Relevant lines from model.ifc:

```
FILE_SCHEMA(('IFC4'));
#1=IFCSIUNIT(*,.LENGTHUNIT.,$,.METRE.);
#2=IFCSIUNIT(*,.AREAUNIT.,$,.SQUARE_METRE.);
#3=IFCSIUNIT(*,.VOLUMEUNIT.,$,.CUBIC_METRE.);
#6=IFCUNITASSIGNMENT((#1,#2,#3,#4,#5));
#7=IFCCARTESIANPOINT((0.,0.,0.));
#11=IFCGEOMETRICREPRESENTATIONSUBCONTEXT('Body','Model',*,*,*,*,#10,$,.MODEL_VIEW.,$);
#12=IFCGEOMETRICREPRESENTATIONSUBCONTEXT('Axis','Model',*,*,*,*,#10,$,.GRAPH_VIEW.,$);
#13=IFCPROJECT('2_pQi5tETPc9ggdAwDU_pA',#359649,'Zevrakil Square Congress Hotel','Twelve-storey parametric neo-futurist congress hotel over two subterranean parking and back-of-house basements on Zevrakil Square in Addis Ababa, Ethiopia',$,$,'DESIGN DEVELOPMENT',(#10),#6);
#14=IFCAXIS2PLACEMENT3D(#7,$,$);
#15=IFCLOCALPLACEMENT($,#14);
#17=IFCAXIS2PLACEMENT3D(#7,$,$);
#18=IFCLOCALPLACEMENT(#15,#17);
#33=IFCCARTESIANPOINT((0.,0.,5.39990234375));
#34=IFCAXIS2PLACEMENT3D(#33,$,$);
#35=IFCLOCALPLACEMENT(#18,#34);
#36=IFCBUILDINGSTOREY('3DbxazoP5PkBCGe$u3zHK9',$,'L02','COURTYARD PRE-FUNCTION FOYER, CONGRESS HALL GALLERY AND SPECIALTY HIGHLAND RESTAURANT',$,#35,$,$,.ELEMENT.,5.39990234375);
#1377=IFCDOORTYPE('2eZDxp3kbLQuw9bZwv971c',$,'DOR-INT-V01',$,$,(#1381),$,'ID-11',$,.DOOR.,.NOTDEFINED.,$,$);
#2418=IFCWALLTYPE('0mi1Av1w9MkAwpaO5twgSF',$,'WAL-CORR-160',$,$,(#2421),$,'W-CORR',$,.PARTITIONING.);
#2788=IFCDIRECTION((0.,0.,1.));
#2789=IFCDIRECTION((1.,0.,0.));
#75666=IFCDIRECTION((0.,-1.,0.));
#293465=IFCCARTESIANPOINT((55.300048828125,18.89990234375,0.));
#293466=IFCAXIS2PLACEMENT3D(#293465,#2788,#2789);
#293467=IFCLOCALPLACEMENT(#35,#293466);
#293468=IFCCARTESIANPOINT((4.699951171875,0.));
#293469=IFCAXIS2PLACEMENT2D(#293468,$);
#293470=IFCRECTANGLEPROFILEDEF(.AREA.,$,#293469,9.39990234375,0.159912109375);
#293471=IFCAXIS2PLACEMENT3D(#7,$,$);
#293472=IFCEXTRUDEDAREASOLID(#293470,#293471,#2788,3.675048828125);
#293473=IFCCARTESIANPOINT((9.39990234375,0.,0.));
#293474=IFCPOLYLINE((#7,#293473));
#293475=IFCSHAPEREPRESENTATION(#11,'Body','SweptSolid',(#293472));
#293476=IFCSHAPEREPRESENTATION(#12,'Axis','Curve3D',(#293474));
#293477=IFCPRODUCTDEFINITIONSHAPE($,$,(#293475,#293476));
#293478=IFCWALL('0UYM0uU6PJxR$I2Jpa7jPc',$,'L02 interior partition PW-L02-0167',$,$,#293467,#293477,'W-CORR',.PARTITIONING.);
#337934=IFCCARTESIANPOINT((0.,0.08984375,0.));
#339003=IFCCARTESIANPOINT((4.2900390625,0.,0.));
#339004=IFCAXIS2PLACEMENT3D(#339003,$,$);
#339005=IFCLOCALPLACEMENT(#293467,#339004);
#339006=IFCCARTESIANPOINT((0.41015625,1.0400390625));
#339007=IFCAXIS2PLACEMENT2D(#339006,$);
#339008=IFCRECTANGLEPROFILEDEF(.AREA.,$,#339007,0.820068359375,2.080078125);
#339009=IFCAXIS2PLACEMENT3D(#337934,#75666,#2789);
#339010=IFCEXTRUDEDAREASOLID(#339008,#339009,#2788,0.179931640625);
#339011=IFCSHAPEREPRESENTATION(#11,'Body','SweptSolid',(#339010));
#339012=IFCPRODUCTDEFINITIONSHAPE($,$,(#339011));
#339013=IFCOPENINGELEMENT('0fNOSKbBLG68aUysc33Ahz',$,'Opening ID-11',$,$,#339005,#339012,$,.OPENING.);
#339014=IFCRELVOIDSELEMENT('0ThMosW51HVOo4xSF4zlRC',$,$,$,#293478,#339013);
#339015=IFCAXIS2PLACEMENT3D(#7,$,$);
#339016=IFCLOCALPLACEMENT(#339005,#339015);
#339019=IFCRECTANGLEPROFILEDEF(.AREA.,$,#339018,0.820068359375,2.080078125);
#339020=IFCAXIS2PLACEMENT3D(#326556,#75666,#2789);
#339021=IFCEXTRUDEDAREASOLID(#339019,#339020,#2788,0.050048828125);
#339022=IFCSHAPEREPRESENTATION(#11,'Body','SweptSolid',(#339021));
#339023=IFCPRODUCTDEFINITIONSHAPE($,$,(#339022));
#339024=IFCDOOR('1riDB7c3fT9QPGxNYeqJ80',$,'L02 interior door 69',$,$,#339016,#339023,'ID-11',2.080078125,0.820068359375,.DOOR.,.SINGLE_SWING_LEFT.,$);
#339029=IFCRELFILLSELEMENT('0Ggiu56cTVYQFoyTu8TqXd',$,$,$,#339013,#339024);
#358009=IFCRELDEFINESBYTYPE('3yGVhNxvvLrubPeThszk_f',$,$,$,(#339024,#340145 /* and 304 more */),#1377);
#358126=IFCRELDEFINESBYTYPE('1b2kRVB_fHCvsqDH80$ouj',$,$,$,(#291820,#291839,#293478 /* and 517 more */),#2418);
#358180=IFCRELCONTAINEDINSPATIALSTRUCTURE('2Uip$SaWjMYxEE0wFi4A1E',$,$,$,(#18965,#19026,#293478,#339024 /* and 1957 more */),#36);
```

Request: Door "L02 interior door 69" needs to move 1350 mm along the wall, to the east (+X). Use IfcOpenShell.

```python
import ifcopenshell
import ifcopenshell.api.geometry
import ifcopenshell.util.placement

model = ifcopenshell.open("model.ifc")

door = model.by_id(339024)
opening = door.FillsVoids[0].RelatingOpeningElement
wall = opening.VoidsElements[0].RelatingBuildingElement

wall_matrix = ifcopenshell.util.placement.get_local_placement(wall.ObjectPlacement)
shift = wall_matrix[:3, 0] * 1.35
before = ifcopenshell.util.placement.get_local_placement(door.ObjectPlacement)[:3, 3].copy()

# The door is placed relative to its opening, so it follows when the opening moves.
matrix = ifcopenshell.util.placement.get_local_placement(opening.ObjectPlacement)
matrix[:3, 3] += shift
ifcopenshell.api.geometry.edit_object_placement(
    model, product=opening, matrix=matrix, is_si=False, should_transform_children=True
)

after = ifcopenshell.util.placement.get_local_placement(door.ObjectPlacement)[:3, 3]
print("door moved by", (after - before).round(3) + 0.0)

model.write("model_edited.ifc")
```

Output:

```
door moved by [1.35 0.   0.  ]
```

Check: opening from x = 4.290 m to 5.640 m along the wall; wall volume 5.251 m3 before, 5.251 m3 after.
